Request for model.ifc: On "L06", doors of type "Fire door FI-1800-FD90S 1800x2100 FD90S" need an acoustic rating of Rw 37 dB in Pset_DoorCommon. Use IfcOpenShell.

First a look at what the model holds.

```python
import ifcopenshell
import ifcopenshell.util.element

model = ifcopenshell.open("model.ifc")
print(model.schema)
storey = next(s for s in model.by_type("IfcBuildingStorey") if s.Name == "L06")
doors = [e for e in ifcopenshell.util.element.get_decomposition(storey) if e.is_a("IfcDoor")]
seen = {}
for e in doors:
    element_type = ifcopenshell.util.element.get_type(e)
    key = (element_type.Name if element_type != e and element_type else None, ifcopenshell.util.element.get_pset(e, "Pset_DoorCommon", "AcousticRating"))
    seen[key] = seen.get(key, 0) + 1
for (name, value), count in sorted(seen.items(), key=str):
    print(count, "x", name, "|", value)
```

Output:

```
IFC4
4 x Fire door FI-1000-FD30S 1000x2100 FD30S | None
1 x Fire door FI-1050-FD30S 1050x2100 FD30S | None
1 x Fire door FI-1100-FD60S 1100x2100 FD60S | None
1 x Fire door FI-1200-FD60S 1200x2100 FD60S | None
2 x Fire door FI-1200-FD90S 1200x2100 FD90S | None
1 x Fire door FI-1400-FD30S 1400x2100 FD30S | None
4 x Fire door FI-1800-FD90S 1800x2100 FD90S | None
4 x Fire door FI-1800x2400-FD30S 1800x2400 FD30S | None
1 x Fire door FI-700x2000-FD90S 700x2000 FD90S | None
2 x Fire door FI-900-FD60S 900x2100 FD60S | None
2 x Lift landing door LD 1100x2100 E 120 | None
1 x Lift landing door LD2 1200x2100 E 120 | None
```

```python
import ifcopenshell
import ifcopenshell.api.pset
import ifcopenshell.util.element

model = ifcopenshell.open("model.ifc")

storey = next(s for s in model.by_type("IfcBuildingStorey") if s.Name == "L06")
doors = [e for e in ifcopenshell.util.element.get_decomposition(storey) if e.is_a("IfcDoor")]

count = 0
for e in doors:
    element_type = ifcopenshell.util.element.get_type(e)
    if element_type in (None, e) or element_type.Name != "Fire door FI-1800-FD90S 1800x2100 FD90S":
        continue
    # add_pset returns the element's existing set when there is one.
    pset = ifcopenshell.api.pset.add_pset(model, product=e, name="Pset_DoorCommon")
    ifcopenshell.api.pset.edit_pset(model, pset=pset, properties={"AcousticRating": "Rw 37 dB"})
    count += 1

print(count, "doors updated")

model.write("model_edited.ifc")
```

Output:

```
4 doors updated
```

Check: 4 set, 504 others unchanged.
